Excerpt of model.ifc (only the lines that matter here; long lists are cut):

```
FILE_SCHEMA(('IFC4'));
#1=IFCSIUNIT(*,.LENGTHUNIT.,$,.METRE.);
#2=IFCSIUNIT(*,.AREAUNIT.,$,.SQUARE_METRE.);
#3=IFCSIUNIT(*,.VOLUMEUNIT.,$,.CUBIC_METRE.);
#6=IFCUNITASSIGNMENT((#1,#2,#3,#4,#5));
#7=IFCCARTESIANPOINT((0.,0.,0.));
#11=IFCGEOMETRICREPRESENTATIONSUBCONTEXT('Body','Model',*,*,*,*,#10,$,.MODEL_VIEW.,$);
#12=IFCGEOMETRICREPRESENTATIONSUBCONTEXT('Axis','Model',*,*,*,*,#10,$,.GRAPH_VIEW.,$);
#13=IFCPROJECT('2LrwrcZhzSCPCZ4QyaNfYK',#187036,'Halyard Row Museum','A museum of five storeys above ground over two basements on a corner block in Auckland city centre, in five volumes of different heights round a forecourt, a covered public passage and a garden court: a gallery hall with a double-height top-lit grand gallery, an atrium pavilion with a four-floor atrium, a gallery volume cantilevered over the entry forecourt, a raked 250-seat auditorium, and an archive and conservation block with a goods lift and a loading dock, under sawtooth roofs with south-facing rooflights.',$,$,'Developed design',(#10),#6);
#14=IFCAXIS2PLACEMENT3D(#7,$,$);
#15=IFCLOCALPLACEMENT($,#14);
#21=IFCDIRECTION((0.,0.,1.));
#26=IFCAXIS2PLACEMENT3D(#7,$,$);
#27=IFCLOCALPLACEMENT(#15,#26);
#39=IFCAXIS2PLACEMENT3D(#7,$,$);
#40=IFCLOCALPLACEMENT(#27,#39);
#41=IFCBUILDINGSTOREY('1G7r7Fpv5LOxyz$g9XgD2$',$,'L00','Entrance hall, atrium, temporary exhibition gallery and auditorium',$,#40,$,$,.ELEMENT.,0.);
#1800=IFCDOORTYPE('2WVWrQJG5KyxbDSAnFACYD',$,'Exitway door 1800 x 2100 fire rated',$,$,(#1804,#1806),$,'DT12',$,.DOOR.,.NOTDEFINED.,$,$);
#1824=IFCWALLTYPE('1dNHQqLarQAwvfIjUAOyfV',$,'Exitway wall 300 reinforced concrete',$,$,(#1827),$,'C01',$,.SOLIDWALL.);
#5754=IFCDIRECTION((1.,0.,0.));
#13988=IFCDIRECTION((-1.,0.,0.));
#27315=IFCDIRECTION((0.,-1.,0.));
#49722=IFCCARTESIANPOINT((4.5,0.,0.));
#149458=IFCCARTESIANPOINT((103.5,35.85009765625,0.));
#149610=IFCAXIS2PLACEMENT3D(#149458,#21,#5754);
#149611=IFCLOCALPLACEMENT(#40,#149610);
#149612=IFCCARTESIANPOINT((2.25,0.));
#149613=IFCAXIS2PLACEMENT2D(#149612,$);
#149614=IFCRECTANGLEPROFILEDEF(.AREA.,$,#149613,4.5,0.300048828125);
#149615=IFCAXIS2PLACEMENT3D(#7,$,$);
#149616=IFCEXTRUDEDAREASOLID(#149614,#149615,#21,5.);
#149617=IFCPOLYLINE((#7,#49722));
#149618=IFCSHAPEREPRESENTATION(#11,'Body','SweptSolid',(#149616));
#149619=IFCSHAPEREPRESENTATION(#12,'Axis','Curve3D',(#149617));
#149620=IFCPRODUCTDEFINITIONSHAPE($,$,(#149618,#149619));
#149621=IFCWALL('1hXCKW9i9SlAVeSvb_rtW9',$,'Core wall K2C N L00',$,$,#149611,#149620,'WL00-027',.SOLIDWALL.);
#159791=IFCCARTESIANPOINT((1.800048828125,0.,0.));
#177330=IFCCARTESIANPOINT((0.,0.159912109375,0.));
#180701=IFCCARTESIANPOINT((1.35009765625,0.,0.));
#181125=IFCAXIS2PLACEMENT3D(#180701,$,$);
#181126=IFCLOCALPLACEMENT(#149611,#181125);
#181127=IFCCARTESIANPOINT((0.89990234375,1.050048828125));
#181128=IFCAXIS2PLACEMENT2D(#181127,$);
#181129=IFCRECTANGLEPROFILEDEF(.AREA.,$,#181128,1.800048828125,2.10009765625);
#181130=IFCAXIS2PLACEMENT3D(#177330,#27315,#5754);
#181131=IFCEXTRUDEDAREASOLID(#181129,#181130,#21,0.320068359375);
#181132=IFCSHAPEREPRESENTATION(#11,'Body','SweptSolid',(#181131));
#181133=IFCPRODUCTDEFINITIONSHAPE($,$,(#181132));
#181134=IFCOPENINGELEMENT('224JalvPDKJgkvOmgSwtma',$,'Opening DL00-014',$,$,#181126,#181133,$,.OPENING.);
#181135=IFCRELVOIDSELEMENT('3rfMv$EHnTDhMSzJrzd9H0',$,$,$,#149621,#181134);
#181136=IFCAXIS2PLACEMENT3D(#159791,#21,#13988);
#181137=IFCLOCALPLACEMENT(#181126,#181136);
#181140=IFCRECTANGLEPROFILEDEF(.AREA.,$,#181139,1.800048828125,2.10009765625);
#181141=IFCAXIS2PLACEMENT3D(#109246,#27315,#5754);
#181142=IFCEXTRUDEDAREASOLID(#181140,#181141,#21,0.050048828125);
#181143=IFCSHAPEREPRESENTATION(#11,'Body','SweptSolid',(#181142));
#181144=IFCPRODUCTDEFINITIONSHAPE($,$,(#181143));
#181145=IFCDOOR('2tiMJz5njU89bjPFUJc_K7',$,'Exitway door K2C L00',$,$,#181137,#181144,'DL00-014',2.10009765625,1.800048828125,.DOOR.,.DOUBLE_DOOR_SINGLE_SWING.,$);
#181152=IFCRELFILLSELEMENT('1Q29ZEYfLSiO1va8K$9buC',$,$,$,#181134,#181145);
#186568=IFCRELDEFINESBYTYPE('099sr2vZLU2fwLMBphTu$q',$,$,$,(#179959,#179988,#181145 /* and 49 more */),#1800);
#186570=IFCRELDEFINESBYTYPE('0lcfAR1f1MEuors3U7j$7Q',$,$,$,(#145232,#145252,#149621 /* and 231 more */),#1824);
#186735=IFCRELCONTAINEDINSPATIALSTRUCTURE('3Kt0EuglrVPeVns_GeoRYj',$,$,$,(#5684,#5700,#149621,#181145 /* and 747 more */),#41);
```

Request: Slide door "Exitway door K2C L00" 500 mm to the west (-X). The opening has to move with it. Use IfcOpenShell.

```python
import ifcopenshell
import ifcopenshell.api.geometry
import ifcopenshell.util.placement
import ifcopenshell.util.unit

model = ifcopenshell.open("model.ifc")
unit_scale = ifcopenshell.util.unit.calculate_unit_scale(model)

door = model.by_id(181145)
opening = door.FillsVoids[0].RelatingOpeningElement
wall = opening.VoidsElements[0].RelatingBuildingElement

wall_matrix = ifcopenshell.util.placement.get_local_placement(wall.ObjectPlacement)
shift = wall_matrix[:3, 0] * -0.5 / unit_scale
before = ifcopenshell.util.placement.get_local_placement(door.ObjectPlacement)[:3, 3].copy()

# The door is placed relative to its opening, so it follows when the opening moves.
matrix = ifcopenshell.util.placement.get_local_placement(opening.ObjectPlacement)
matrix[:3, 3] += shift
ifcopenshell.api.geometry.edit_object_placement(
    model, product=opening, matrix=matrix, is_si=False, should_transform_children=True
)

after = ifcopenshell.util.placement.get_local_placement(door.ObjectPlacement)[:3, 3]
print("door moved by", (after - before).round(3) + 0.0)

model.write("model_v2.ifc")
```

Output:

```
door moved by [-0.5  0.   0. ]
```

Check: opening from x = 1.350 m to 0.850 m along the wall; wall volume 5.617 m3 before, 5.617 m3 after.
